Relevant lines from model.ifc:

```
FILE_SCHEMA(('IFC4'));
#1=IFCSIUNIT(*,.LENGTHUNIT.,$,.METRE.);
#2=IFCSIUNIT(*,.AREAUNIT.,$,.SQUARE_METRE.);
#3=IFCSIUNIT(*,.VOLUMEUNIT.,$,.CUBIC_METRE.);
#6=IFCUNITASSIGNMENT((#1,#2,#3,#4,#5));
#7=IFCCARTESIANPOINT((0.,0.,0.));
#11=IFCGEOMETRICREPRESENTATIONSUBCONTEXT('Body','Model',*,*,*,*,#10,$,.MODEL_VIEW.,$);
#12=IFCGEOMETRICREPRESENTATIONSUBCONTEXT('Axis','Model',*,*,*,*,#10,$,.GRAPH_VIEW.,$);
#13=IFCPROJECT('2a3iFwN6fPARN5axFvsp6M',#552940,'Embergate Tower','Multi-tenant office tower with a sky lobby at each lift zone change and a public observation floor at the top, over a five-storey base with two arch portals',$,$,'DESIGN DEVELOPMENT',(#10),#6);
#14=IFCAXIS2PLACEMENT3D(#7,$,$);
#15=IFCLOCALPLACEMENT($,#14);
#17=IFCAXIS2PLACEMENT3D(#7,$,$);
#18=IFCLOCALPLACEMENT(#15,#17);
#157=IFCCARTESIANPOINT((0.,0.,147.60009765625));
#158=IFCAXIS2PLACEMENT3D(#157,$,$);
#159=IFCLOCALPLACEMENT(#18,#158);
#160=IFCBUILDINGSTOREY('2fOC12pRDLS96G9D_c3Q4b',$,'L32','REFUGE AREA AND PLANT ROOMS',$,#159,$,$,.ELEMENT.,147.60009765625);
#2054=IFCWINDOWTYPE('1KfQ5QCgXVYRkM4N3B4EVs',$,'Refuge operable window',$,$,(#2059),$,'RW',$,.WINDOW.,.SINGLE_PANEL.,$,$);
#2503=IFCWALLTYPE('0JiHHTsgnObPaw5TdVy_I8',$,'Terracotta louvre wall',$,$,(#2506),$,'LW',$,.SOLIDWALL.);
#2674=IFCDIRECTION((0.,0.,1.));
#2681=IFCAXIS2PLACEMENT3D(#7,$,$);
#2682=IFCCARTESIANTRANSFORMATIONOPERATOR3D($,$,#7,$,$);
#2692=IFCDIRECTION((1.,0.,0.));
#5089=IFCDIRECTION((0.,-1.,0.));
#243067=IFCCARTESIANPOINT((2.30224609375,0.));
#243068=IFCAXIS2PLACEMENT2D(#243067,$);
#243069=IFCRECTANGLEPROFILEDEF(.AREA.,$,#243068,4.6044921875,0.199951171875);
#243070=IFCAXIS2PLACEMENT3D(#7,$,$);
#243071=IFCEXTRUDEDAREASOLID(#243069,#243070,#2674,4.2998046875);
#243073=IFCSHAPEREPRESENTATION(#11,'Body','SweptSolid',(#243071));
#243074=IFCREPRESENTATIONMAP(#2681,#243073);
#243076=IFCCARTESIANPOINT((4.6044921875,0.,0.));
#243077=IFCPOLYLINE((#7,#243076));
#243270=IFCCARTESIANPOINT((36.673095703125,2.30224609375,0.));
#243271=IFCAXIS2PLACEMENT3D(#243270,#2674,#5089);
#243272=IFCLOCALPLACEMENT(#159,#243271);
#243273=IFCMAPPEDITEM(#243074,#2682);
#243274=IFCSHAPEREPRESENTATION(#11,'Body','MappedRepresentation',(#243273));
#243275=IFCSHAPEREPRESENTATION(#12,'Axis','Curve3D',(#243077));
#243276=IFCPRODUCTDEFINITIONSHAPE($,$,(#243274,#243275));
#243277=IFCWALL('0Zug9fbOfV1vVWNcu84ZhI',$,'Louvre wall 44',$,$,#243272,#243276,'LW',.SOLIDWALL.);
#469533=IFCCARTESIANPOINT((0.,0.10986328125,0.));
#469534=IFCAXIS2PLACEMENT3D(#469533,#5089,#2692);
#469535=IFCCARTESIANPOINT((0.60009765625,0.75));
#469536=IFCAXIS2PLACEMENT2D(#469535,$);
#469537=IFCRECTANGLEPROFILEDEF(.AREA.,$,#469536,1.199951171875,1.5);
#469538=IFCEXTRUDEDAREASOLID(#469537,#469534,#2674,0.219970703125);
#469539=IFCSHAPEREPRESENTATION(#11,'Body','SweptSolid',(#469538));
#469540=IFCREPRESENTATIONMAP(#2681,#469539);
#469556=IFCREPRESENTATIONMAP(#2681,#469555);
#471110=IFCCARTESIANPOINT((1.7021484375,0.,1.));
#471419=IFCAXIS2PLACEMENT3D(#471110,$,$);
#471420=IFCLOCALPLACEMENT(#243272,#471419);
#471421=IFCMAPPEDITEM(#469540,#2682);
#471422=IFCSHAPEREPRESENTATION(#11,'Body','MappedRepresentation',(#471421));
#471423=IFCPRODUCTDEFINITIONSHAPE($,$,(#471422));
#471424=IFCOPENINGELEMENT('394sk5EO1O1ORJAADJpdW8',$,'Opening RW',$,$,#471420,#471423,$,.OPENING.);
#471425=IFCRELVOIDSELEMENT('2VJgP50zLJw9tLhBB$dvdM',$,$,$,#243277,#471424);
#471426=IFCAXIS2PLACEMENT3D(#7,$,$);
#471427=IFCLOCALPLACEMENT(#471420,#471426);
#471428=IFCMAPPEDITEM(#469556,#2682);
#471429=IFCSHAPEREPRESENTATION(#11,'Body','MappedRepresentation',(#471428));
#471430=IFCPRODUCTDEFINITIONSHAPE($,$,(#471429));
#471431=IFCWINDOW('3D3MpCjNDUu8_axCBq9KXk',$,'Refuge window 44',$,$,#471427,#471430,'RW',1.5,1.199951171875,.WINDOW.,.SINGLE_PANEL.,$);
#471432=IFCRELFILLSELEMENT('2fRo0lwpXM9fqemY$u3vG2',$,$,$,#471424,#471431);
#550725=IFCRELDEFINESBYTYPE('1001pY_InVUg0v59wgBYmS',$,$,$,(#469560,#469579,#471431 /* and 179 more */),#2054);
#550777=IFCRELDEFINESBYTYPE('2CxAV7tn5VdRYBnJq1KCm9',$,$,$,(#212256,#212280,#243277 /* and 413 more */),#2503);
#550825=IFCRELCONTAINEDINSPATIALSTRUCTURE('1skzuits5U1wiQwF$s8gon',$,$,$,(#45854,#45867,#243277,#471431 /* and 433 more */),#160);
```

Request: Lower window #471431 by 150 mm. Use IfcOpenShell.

```python
import numpy as np
import ifcopenshell
import ifcopenshell.api.geometry
import ifcopenshell.util.placement
import ifcopenshell.util.unit

model = ifcopenshell.open("model.ifc")
unit_scale = ifcopenshell.util.unit.calculate_unit_scale(model)

window = model.by_guid("3D3MpCjNDUu8_axCBq9KXk")
opening = window.FillsVoids[0].RelatingOpeningElement
dz = -0.15

shift = np.array([0.0, 0.0, dz])
# The window is placed relative to its opening, so it follows when the opening moves.
matrix = ifcopenshell.util.placement.get_local_placement(opening.ObjectPlacement)
matrix[:3, 3] += shift
ifcopenshell.api.geometry.edit_object_placement(
    model, product=opening, matrix=matrix, is_si=False, should_transform_children=True
)

print(f"moved by {dz * unit_scale:+.3f} m")

model.write("model-out.ifc")
```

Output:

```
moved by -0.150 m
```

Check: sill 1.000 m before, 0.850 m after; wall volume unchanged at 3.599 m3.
